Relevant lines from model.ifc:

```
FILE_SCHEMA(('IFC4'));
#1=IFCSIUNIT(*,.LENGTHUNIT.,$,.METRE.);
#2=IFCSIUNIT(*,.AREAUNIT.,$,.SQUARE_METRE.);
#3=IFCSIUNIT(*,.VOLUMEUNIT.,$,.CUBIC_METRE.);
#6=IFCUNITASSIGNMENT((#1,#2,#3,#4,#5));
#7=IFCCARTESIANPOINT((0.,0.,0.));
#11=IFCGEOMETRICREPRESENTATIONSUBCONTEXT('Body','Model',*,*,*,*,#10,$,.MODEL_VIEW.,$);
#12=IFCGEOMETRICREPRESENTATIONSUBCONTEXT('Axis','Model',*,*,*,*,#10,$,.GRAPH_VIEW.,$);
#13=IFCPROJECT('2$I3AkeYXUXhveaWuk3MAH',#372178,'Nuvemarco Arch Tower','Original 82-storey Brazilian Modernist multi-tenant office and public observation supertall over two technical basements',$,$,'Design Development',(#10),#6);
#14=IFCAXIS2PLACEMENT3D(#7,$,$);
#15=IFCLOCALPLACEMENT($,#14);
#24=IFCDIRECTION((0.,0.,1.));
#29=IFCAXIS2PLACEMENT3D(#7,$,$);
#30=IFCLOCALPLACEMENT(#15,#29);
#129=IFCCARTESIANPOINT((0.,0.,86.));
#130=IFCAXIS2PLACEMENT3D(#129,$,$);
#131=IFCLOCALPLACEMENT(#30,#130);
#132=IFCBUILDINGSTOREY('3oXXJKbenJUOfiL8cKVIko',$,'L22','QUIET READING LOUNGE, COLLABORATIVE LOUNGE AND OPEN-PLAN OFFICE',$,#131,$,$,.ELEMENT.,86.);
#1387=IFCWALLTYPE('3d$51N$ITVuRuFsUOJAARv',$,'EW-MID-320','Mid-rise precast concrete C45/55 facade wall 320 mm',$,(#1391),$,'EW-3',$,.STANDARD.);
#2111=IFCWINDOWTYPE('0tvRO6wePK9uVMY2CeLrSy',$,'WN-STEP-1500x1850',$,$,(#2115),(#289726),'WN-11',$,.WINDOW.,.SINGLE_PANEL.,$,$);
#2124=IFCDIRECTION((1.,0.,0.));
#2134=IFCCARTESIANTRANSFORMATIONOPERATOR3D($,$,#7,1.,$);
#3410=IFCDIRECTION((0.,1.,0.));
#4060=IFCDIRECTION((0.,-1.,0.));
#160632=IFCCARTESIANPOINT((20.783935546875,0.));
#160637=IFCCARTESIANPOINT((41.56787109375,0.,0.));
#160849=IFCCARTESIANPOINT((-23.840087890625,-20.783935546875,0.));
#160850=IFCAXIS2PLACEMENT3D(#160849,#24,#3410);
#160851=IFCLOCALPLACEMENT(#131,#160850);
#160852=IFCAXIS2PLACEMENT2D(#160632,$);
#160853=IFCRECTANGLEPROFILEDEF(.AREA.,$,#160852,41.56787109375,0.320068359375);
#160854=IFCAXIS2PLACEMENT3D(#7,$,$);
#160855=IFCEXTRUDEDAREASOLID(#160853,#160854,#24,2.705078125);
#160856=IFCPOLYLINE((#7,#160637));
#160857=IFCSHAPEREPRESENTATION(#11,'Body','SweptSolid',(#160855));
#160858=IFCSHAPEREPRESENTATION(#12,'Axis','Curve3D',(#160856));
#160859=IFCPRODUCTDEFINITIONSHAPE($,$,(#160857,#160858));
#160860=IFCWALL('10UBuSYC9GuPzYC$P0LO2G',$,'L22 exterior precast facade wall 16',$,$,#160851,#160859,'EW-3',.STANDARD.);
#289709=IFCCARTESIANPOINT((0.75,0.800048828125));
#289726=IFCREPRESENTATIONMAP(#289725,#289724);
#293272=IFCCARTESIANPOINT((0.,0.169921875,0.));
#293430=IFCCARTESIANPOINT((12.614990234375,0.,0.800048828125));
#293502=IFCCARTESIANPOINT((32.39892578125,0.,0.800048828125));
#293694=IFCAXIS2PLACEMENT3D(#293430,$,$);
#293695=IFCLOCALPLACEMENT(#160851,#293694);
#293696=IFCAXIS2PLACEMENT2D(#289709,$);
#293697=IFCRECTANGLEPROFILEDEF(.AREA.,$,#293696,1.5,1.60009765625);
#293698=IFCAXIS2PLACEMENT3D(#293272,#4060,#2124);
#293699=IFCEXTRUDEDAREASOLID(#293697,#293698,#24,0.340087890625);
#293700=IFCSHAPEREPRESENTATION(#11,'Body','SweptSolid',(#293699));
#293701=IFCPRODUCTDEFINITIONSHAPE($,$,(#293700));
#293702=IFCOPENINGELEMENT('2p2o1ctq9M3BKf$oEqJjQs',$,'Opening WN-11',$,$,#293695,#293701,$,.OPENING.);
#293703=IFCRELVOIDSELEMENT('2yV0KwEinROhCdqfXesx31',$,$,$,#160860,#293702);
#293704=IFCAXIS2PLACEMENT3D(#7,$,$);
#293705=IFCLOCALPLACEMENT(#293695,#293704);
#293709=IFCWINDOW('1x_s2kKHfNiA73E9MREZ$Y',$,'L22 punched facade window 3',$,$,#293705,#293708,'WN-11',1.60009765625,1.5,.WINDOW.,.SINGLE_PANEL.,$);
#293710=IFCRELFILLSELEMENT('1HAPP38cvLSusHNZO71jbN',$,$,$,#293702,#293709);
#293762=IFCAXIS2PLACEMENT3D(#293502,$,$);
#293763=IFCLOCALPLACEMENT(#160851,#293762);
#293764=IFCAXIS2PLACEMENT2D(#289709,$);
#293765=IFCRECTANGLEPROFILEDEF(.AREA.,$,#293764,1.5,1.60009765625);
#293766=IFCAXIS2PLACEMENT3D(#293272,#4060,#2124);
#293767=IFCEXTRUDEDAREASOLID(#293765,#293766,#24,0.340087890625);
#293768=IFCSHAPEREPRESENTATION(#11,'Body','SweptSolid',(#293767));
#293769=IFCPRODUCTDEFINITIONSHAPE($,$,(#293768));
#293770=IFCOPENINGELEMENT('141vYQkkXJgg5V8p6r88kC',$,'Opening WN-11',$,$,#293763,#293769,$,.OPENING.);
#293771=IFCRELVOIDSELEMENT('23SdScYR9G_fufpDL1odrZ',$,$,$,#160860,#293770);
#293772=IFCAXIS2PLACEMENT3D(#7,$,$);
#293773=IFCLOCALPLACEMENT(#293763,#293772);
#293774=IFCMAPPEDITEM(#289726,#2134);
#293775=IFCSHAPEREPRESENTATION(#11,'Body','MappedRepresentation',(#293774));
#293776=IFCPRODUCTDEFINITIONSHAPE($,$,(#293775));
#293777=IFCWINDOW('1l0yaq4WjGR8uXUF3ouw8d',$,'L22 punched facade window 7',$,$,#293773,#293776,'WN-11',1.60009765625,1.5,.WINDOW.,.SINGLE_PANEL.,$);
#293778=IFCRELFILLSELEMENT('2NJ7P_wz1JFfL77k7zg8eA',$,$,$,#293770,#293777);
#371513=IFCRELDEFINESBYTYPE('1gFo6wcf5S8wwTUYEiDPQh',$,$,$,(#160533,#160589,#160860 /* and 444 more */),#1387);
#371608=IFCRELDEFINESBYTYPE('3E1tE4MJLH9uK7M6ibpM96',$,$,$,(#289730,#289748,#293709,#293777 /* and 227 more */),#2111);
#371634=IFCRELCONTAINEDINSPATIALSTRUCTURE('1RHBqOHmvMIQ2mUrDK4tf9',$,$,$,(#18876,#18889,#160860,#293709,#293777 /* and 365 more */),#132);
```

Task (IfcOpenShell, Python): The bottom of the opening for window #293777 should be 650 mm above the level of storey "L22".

```python
import numpy as np
import ifcopenshell
import ifcopenshell.api.geometry
import ifcopenshell.geom
import ifcopenshell.util.element
import ifcopenshell.util.placement
import ifcopenshell.util.shape
import ifcopenshell.util.unit

model = ifcopenshell.open("model.ifc")
unit_scale = ifcopenshell.util.unit.calculate_unit_scale(model)

window = model.by_guid("1l0yaq4WjGR8uXUF3ouw8d")
opening = window.FillsVoids[0].RelatingOpeningElement
storey = ifcopenshell.util.element.get_container(window, ifc_class="IfcBuildingStorey")
level = ifcopenshell.util.placement.get_local_placement(storey.ObjectPlacement)[2, 3]

# The opening's origin need not be at the sill, so measure its lowest point.
shape = ifcopenshell.geom.create_shape(ifcopenshell.geom.settings(), opening)
bottom = ifcopenshell.util.shape.get_shape_bottom_elevation(shape, shape.geometry) / unit_scale
dz = level + 0.65 - bottom

shift = np.array([0.0, 0.0, dz])
# The window is placed relative to its opening, so it follows when the opening moves.
matrix = ifcopenshell.util.placement.get_local_placement(opening.ObjectPlacement)
matrix[:3, 3] += shift
ifcopenshell.api.geometry.edit_object_placement(
    model, product=opening, matrix=matrix, is_si=False, should_transform_children=True
)

print(f"moved by {dz * unit_scale:+.3f} m")

model.write("model_edited.ifc")
```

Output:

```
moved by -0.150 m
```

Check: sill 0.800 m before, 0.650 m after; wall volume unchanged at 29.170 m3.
